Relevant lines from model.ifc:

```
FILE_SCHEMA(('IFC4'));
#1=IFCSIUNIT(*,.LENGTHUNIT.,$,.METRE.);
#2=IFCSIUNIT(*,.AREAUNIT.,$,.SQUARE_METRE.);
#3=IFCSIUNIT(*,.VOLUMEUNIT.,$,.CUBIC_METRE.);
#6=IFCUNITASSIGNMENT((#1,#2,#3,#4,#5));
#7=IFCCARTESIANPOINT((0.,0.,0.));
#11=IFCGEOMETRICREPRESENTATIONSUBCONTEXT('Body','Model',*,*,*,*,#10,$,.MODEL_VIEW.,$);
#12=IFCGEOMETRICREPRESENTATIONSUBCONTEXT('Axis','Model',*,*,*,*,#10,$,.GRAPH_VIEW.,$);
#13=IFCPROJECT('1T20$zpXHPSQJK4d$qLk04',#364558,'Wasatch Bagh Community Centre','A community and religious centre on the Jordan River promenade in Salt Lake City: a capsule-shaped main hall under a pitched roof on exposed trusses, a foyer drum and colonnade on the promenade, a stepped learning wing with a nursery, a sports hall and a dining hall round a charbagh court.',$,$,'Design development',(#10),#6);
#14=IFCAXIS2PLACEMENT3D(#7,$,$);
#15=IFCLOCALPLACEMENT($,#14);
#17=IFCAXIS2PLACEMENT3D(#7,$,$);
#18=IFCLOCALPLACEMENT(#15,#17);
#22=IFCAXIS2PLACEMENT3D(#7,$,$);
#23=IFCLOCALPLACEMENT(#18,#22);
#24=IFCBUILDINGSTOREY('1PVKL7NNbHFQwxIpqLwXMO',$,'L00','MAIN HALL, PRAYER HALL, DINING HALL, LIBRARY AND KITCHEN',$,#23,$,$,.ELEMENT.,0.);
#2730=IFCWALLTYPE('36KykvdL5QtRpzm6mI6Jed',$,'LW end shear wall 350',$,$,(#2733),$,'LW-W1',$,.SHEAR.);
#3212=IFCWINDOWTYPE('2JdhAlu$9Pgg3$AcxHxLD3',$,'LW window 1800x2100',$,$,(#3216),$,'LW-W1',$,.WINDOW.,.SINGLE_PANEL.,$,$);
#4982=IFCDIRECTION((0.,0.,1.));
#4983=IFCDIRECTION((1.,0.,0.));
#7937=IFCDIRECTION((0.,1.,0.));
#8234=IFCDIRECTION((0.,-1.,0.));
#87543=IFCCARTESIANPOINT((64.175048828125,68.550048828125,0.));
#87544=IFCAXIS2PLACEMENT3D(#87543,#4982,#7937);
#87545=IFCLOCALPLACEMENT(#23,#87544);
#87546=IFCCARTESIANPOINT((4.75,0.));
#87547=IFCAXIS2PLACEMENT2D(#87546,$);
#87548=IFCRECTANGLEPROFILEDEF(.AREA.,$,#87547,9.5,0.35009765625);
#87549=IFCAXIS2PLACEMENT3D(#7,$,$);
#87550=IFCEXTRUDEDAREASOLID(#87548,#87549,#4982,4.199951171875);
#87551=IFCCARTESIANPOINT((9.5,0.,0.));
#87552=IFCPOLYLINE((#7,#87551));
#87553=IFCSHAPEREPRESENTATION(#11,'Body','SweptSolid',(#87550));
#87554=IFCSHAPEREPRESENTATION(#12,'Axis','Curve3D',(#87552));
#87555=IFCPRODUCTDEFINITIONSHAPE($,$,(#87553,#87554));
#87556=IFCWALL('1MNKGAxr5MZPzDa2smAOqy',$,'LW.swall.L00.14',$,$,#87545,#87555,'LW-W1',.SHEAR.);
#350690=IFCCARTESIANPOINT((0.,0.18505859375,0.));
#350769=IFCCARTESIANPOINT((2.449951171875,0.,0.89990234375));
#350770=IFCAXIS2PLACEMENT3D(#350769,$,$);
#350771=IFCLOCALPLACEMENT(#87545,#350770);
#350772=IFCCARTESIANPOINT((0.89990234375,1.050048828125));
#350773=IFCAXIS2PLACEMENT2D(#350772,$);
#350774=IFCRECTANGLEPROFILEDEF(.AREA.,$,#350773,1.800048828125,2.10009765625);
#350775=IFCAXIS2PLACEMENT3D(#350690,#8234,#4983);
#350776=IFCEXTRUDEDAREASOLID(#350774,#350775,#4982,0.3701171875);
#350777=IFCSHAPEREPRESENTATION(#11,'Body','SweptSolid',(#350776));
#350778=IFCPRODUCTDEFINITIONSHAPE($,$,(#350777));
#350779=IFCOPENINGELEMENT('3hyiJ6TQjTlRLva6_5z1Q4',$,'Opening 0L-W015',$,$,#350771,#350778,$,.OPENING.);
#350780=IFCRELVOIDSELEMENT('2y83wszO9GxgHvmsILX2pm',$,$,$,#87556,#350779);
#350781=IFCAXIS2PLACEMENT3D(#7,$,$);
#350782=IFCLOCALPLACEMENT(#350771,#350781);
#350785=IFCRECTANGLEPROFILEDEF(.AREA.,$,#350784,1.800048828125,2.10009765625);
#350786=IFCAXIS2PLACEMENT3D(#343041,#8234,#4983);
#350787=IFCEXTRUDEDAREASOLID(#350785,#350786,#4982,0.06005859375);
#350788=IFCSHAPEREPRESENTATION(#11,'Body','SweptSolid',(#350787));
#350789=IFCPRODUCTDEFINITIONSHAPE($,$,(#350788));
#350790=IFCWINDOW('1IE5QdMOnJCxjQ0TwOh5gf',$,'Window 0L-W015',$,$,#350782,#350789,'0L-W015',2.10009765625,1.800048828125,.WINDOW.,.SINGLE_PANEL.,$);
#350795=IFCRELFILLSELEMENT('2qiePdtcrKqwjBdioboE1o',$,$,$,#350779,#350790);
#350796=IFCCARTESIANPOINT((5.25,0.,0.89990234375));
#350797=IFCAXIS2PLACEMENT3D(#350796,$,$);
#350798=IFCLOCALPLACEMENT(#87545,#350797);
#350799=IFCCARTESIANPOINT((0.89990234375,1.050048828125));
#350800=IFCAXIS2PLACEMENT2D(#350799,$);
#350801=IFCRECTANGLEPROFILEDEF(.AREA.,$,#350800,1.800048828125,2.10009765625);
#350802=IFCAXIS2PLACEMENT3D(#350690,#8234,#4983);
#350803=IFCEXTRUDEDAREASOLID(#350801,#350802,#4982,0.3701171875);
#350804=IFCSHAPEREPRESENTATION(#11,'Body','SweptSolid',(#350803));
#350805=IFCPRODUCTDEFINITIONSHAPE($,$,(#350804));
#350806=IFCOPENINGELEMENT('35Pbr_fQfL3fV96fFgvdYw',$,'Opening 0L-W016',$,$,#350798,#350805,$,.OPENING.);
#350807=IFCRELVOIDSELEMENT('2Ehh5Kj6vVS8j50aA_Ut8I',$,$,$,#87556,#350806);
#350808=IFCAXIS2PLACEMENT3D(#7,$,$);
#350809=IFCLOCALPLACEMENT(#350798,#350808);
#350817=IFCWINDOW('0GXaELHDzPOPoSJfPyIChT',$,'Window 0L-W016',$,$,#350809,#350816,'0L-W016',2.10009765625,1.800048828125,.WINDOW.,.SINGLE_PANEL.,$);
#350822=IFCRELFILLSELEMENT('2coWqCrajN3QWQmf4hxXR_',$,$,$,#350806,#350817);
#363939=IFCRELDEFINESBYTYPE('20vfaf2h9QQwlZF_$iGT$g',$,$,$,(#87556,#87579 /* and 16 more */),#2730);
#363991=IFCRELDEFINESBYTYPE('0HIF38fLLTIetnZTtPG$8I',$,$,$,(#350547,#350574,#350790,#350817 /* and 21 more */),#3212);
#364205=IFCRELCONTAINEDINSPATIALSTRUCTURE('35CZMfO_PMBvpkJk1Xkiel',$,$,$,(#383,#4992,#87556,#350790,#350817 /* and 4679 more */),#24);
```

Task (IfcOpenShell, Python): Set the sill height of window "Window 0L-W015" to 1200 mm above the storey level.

```python
import numpy as np
import ifcopenshell
import ifcopenshell.api.geometry
import ifcopenshell.geom
import ifcopenshell.util.element
import ifcopenshell.util.placement
import ifcopenshell.util.shape
import ifcopenshell.util.unit

model = ifcopenshell.open("model.ifc")
unit_scale = ifcopenshell.util.unit.calculate_unit_scale(model)

window = model.by_guid("1IE5QdMOnJCxjQ0TwOh5gf")
opening = window.FillsVoids[0].RelatingOpeningElement
storey = ifcopenshell.util.element.get_container(window, ifc_class="IfcBuildingStorey")
level = ifcopenshell.util.placement.get_local_placement(storey.ObjectPlacement)[2, 3]

# The opening's origin need not be at the sill, so measure its lowest point.
shape = ifcopenshell.geom.create_shape(ifcopenshell.geom.settings(), opening)
bottom = ifcopenshell.util.shape.get_shape_bottom_elevation(shape, shape.geometry) / unit_scale
dz = level + 1.2 - bottom

shift = np.array([0.0, 0.0, dz])
# The window is placed relative to its opening, so it follows when the opening moves.
matrix = ifcopenshell.util.placement.get_local_placement(opening.ObjectPlacement)
matrix[:3, 3] += shift
ifcopenshell.api.geometry.edit_object_placement(
    model, product=opening, matrix=matrix, is_si=False, should_transform_children=True
)

print(f"moved by {dz * unit_scale:+.3f} m")

model.write("model_edited.ifc")
```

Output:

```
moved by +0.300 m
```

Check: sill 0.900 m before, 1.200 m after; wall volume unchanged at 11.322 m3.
